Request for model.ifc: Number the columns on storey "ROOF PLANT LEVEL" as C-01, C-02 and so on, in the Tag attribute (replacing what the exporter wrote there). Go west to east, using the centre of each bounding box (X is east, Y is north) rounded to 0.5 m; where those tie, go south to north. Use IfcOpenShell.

First a look at what the model holds.

```python
import ifcopenshell
import ifcopenshell.util.element
import ifcopenshell.util.placement

model = ifcopenshell.open("model.ifc")
print(model.schema)
storey = next(s for s in model.by_type("IfcBuildingStorey") if s.Name == "ROOF PLANT LEVEL")
columns = [e for e in ifcopenshell.util.element.get_decomposition(storey) if e.is_a("IfcColumn")]
for e in sorted(columns, key=lambda e: e.id()):
    origin = ifcopenshell.util.placement.get_local_placement(e.ObjectPlacement)[:3, 3]
    print(e.id(), e.Tag, e.Name, origin.round(2) + 0.0, sep=" | ")
```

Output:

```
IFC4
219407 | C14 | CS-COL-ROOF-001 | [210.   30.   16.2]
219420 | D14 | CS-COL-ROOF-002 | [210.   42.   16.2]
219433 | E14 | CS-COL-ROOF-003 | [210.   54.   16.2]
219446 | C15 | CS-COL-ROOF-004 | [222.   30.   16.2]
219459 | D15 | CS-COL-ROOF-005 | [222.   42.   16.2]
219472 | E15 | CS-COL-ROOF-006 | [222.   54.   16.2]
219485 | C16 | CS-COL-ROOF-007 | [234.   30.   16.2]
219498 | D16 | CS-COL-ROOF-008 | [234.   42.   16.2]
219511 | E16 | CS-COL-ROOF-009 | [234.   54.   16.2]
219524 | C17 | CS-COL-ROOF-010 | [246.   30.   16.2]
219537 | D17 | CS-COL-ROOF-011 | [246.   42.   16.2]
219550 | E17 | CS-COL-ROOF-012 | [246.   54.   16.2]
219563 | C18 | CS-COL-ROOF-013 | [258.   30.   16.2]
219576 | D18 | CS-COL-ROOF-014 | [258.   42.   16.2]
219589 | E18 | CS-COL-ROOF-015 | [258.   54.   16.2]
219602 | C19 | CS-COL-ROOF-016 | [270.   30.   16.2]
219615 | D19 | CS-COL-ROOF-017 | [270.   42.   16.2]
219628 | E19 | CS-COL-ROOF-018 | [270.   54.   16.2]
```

```python
import ifcopenshell
import ifcopenshell.geom
import ifcopenshell.util.element
import ifcopenshell.util.shape

model = ifcopenshell.open("model.ifc")
settings = ifcopenshell.geom.settings()
settings.set("use-world-coords", True)


def centre(element):
    shape = ifcopenshell.geom.create_shape(settings, element)
    return ifcopenshell.util.shape.get_bbox_centroid(shape.geometry)


storey = next(s for s in model.by_type("IfcBuildingStorey") if s.Name == "ROOF PLANT LEVEL")
columns = [e for e in ifcopenshell.util.element.get_decomposition(storey) if e.is_a("IfcColumn")]

# Insertion points can sit at a corner or the storey origin, so sort by the geometry (in metres).
centres = {e: centre(e) for e in columns}
columns.sort(key=lambda e: (round(centres[e][0] / 0.5), centres[e][1]))

for i, e in enumerate(columns, start=1):
    number = f"C-{i:02d}"
    e.Tag = number
    print(e.id(), number)

model.write("model_v2.ifc")
```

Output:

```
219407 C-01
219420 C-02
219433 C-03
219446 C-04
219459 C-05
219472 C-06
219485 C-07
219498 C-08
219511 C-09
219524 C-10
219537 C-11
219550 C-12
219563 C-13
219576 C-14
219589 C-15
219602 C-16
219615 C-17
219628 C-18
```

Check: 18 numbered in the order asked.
